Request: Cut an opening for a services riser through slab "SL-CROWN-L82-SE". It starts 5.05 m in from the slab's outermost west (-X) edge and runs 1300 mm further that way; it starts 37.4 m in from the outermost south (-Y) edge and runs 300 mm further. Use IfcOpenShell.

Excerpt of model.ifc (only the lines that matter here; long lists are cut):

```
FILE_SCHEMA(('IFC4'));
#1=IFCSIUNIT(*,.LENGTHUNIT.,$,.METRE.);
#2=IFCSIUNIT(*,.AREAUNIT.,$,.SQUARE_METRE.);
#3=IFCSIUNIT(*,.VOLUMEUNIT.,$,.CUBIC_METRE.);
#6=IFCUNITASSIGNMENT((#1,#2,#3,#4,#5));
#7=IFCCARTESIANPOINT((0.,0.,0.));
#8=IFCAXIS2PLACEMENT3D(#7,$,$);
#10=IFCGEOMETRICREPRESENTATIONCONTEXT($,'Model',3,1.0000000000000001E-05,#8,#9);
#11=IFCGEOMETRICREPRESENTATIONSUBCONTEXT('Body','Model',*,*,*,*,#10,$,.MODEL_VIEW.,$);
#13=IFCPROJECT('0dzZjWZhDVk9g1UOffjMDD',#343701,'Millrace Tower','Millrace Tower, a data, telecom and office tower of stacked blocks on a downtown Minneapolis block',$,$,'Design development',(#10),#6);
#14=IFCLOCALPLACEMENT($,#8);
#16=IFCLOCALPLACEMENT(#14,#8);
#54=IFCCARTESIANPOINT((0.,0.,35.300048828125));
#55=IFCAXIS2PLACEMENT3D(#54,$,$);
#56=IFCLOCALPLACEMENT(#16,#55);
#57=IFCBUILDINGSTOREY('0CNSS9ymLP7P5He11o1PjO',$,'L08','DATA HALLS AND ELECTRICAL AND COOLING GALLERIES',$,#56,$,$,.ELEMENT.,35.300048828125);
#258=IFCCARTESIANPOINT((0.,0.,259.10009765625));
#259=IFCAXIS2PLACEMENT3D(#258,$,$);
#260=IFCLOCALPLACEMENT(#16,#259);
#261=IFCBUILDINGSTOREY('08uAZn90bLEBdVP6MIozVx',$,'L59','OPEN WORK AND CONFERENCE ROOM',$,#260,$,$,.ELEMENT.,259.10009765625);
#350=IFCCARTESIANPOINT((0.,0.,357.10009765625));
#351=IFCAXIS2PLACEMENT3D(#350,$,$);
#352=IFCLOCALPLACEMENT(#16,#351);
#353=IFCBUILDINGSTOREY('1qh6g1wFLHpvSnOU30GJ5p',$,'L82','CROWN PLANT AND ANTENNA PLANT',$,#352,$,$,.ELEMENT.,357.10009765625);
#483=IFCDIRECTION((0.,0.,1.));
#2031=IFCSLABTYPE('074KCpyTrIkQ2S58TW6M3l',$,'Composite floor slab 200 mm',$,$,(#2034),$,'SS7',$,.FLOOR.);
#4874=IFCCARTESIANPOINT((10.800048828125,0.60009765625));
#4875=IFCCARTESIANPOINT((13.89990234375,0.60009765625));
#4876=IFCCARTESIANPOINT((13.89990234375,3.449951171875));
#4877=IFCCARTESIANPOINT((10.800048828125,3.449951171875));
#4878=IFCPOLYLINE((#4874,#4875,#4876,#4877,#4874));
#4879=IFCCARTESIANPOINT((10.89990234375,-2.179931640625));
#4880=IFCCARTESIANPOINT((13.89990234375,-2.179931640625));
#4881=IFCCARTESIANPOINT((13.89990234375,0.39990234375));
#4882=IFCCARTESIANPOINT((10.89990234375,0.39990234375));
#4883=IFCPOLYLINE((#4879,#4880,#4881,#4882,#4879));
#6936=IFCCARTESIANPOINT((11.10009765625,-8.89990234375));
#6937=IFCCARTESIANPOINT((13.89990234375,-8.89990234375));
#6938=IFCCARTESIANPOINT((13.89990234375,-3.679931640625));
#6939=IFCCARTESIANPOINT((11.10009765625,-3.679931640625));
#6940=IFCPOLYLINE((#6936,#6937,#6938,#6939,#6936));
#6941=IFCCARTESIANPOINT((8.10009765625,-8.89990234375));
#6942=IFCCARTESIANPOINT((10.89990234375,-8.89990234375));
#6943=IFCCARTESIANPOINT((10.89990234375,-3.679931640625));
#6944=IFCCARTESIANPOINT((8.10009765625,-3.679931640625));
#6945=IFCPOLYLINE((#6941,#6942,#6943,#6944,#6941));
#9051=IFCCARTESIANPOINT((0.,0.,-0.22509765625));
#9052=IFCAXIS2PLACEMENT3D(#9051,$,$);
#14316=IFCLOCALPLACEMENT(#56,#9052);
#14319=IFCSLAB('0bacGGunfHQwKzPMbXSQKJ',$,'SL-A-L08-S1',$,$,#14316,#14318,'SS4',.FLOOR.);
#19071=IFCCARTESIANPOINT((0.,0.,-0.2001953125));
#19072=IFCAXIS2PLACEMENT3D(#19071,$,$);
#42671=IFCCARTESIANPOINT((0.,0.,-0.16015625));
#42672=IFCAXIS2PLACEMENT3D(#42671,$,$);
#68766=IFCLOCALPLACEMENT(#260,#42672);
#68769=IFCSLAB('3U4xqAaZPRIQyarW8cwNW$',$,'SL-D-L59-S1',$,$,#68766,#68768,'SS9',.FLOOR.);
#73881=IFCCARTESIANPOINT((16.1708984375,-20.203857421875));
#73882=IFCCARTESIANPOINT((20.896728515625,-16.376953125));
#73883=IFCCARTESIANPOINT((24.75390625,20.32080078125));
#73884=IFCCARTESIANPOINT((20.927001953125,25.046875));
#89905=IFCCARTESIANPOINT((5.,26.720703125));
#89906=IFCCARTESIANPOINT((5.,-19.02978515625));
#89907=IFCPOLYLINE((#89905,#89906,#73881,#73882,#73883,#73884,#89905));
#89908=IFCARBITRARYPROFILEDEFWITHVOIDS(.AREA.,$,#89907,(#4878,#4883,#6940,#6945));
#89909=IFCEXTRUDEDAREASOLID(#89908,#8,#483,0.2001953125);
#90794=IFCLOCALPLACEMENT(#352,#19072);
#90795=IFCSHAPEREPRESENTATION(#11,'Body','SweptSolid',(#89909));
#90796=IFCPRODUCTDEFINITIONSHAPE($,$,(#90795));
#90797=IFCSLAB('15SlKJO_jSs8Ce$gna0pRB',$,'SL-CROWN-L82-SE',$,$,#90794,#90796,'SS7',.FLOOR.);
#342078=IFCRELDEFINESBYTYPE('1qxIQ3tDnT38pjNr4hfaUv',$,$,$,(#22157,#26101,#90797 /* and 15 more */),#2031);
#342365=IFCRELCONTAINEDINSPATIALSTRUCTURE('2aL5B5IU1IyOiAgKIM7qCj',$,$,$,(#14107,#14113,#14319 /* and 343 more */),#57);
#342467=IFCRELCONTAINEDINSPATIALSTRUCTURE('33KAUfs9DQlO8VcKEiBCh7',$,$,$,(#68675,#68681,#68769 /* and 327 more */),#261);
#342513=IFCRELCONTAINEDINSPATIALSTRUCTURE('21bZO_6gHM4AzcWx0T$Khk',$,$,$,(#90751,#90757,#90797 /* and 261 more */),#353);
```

```python
import numpy as np
import ifcopenshell
import ifcopenshell.api.feature
import ifcopenshell.api.geometry
import ifcopenshell.api.root
import ifcopenshell.geom
import ifcopenshell.util.placement
import ifcopenshell.util.representation
import ifcopenshell.util.shape
import ifcopenshell.util.unit

model = ifcopenshell.open("model.ifc")
unit_scale = ifcopenshell.util.unit.calculate_unit_scale(model)
settings = ifcopenshell.geom.settings()


def volume(element):
    """Net volume in cubic metres, openings subtracted."""
    shape = ifcopenshell.geom.create_shape(settings, element)
    return ifcopenshell.util.shape.get_volume(shape.geometry)


slab = model.by_id(90797)
before = volume(slab)

# Extent in the slab's own axes, in metres. The edges named are its -X and -Y sides.
slab_shape = ifcopenshell.geom.create_shape(settings, slab)
vertices = ifcopenshell.util.shape.get_vertices(slab_shape.geometry)
x_min, y_min, bottom = vertices.min(axis=0)
top = vertices[:, 2].max()

opening = ifcopenshell.api.root.create_entity(model, ifc_class="IfcOpeningElement", name="Services riser opening", predefined_type="OPENING")
context = ifcopenshell.util.representation.get_context(model, "Model", "Body", "MODEL_VIEW")
width, depth = 1.3, 0.3
outline = [(0.0, 0.0), (width, 0.0), (width, depth), (0.0, depth), (0.0, 0.0)]
# Overshoot both faces by 50 mm so the cut is clean.
shape = ifcopenshell.api.geometry.add_slab_representation(
    model, context=context, depth=top - bottom + 0.1, polyline=outline
)
ifcopenshell.api.geometry.assign_representation(model, product=opening, representation=shape)

matrix = ifcopenshell.util.placement.get_local_placement(slab.ObjectPlacement)
matrix[:, 3] = matrix @ np.append(np.array([x_min + 5.05, y_min + 37.4, bottom - 0.05]) / unit_scale, 1.0)
ifcopenshell.api.geometry.edit_object_placement(model, product=opening, matrix=matrix, is_si=False)
ifcopenshell.api.feature.add_feature(model, feature=opening, element=slab)

after = volume(slab)

print(f"slab volume {before:.3f} -> {after:.3f} m3")

model.write("model_edited.ifc")
```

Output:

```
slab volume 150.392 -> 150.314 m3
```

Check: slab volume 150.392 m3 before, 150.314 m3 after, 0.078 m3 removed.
